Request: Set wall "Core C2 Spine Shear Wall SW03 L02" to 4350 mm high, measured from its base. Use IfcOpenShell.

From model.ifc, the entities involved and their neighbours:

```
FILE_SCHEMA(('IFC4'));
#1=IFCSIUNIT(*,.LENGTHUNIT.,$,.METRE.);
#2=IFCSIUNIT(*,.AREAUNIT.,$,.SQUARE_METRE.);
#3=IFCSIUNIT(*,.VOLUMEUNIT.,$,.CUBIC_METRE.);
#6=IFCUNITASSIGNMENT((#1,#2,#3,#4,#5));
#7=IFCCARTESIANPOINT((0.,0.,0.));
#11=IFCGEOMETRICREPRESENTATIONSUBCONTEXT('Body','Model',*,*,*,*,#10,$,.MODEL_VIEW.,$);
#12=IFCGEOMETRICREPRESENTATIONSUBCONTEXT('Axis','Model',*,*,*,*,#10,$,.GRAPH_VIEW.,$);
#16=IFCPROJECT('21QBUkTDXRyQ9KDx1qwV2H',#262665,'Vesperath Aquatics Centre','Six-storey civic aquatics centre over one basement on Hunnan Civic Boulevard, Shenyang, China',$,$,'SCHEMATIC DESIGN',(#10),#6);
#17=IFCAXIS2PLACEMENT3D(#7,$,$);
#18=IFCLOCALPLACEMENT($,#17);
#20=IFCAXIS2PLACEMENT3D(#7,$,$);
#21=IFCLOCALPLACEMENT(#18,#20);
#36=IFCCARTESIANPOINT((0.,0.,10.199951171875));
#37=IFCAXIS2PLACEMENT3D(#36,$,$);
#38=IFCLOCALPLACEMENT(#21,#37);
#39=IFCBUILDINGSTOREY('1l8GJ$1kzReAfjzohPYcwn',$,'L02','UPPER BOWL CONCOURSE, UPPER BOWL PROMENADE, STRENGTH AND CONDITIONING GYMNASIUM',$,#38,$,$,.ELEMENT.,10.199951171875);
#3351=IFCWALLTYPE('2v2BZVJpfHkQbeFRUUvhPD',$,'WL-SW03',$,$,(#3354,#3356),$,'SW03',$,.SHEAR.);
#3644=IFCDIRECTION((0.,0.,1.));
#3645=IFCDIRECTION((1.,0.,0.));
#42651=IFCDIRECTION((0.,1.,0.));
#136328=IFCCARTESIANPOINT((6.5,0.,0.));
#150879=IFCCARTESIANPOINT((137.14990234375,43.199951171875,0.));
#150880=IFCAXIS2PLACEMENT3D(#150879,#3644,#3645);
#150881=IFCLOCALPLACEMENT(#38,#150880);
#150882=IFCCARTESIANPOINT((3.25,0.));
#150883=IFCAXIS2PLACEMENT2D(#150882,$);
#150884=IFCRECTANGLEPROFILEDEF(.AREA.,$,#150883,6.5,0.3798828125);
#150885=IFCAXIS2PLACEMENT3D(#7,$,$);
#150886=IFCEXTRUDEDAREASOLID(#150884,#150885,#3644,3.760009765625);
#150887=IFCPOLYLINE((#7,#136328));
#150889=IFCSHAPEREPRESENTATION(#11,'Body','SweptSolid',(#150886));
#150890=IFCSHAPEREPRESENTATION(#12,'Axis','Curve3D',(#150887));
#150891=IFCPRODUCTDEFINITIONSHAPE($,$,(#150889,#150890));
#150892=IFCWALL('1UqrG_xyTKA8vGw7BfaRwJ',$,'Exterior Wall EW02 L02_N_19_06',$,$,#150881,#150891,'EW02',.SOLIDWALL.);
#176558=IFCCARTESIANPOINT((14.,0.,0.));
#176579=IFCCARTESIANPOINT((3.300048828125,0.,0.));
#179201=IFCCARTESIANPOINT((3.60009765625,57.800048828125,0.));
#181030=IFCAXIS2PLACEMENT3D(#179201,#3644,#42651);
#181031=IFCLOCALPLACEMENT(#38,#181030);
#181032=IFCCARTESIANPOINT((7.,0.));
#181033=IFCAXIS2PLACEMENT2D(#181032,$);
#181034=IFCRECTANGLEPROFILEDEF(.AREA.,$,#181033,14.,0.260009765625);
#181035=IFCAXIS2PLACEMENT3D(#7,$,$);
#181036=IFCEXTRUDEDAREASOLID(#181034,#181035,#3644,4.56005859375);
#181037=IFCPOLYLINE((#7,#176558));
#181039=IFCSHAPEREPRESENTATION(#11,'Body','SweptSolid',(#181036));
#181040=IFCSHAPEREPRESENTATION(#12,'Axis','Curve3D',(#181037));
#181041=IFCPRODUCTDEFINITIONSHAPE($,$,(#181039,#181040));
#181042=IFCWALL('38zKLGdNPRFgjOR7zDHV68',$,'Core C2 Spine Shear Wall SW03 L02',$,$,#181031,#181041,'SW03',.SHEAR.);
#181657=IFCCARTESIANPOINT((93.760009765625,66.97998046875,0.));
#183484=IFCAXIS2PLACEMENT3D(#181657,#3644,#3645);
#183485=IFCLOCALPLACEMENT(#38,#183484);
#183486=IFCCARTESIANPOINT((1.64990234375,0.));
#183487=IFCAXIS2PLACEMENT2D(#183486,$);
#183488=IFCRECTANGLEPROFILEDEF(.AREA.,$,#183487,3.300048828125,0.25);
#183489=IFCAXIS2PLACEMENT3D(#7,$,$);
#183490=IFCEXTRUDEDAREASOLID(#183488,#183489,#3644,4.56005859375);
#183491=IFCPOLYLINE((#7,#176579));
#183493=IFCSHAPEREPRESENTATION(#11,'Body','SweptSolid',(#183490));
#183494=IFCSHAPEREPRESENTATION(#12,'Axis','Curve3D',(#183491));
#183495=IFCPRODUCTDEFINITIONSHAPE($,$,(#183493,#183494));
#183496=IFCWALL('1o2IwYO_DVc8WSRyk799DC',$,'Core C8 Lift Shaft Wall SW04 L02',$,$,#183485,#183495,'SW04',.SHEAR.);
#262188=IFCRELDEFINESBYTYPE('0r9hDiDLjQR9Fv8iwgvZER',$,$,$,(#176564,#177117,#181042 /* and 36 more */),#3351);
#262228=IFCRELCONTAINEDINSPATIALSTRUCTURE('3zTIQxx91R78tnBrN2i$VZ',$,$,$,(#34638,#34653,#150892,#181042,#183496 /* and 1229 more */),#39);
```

```python
import ifcopenshell
import ifcopenshell.geom
import ifcopenshell.util.representation
import ifcopenshell.util.shape
import ifcopenshell.util.unit

model = ifcopenshell.open("model.ifc")
unit_scale = ifcopenshell.util.unit.calculate_unit_scale(model)
settings = ifcopenshell.geom.settings()


def volume(element):
    """Net volume in cubic metres, openings subtracted."""
    shape = ifcopenshell.geom.create_shape(settings, element)
    return ifcopenshell.util.shape.get_volume(shape.geometry)


wall = model.by_guid("38zKLGdNPRFgjOR7zDHV68")
before = volume(wall)

body = ifcopenshell.util.representation.get_representation(wall, "Model", "Body")
solid = body.Items[0]
old_height = solid.Depth
solid.Depth = 4.35 / unit_scale
after = volume(wall)

print(f"height {old_height:g} -> {solid.Depth:g}, volume {before:.3f} -> {after:.3f} m3")

model.write("model_edited.ifc")
```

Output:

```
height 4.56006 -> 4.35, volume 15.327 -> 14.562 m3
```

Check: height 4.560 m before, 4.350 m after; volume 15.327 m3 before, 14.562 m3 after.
